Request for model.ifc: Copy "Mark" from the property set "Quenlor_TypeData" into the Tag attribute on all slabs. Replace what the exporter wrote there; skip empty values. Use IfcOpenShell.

First a look at what the model holds.

```python
import ifcopenshell
import ifcopenshell.util.element

model = ifcopenshell.open("model.ifc")
print(model.schema)
slabs = model.by_type("IfcSlab")
print(len(slabs), "slabs")
for e in slabs[:8]:
    source = ifcopenshell.util.element.get_pset(e, "Quenlor_TypeData", "Mark")
    target = e.Tag
    print(e.id(), repr(source), repr(target), sep=" | ")
```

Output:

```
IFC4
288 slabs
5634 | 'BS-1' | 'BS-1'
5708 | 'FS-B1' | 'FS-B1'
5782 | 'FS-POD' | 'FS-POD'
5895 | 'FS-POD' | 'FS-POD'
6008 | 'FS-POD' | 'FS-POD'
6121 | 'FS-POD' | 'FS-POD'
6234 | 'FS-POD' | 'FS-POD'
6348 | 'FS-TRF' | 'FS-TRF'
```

```python
import ifcopenshell
import ifcopenshell.util.element

model = ifcopenshell.open("model.ifc")

count = 0
for e in model.by_type("IfcSlab"):
    value = ifcopenshell.util.element.get_pset(e, "Quenlor_TypeData", "Mark")
    current = e.Tag
    if not value or not value.strip() or current == value:
        continue
    e.Tag = value
    count += 1

print(count, "slabs updated")

model.write("model_edited.ifc")
```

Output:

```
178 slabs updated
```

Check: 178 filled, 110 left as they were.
